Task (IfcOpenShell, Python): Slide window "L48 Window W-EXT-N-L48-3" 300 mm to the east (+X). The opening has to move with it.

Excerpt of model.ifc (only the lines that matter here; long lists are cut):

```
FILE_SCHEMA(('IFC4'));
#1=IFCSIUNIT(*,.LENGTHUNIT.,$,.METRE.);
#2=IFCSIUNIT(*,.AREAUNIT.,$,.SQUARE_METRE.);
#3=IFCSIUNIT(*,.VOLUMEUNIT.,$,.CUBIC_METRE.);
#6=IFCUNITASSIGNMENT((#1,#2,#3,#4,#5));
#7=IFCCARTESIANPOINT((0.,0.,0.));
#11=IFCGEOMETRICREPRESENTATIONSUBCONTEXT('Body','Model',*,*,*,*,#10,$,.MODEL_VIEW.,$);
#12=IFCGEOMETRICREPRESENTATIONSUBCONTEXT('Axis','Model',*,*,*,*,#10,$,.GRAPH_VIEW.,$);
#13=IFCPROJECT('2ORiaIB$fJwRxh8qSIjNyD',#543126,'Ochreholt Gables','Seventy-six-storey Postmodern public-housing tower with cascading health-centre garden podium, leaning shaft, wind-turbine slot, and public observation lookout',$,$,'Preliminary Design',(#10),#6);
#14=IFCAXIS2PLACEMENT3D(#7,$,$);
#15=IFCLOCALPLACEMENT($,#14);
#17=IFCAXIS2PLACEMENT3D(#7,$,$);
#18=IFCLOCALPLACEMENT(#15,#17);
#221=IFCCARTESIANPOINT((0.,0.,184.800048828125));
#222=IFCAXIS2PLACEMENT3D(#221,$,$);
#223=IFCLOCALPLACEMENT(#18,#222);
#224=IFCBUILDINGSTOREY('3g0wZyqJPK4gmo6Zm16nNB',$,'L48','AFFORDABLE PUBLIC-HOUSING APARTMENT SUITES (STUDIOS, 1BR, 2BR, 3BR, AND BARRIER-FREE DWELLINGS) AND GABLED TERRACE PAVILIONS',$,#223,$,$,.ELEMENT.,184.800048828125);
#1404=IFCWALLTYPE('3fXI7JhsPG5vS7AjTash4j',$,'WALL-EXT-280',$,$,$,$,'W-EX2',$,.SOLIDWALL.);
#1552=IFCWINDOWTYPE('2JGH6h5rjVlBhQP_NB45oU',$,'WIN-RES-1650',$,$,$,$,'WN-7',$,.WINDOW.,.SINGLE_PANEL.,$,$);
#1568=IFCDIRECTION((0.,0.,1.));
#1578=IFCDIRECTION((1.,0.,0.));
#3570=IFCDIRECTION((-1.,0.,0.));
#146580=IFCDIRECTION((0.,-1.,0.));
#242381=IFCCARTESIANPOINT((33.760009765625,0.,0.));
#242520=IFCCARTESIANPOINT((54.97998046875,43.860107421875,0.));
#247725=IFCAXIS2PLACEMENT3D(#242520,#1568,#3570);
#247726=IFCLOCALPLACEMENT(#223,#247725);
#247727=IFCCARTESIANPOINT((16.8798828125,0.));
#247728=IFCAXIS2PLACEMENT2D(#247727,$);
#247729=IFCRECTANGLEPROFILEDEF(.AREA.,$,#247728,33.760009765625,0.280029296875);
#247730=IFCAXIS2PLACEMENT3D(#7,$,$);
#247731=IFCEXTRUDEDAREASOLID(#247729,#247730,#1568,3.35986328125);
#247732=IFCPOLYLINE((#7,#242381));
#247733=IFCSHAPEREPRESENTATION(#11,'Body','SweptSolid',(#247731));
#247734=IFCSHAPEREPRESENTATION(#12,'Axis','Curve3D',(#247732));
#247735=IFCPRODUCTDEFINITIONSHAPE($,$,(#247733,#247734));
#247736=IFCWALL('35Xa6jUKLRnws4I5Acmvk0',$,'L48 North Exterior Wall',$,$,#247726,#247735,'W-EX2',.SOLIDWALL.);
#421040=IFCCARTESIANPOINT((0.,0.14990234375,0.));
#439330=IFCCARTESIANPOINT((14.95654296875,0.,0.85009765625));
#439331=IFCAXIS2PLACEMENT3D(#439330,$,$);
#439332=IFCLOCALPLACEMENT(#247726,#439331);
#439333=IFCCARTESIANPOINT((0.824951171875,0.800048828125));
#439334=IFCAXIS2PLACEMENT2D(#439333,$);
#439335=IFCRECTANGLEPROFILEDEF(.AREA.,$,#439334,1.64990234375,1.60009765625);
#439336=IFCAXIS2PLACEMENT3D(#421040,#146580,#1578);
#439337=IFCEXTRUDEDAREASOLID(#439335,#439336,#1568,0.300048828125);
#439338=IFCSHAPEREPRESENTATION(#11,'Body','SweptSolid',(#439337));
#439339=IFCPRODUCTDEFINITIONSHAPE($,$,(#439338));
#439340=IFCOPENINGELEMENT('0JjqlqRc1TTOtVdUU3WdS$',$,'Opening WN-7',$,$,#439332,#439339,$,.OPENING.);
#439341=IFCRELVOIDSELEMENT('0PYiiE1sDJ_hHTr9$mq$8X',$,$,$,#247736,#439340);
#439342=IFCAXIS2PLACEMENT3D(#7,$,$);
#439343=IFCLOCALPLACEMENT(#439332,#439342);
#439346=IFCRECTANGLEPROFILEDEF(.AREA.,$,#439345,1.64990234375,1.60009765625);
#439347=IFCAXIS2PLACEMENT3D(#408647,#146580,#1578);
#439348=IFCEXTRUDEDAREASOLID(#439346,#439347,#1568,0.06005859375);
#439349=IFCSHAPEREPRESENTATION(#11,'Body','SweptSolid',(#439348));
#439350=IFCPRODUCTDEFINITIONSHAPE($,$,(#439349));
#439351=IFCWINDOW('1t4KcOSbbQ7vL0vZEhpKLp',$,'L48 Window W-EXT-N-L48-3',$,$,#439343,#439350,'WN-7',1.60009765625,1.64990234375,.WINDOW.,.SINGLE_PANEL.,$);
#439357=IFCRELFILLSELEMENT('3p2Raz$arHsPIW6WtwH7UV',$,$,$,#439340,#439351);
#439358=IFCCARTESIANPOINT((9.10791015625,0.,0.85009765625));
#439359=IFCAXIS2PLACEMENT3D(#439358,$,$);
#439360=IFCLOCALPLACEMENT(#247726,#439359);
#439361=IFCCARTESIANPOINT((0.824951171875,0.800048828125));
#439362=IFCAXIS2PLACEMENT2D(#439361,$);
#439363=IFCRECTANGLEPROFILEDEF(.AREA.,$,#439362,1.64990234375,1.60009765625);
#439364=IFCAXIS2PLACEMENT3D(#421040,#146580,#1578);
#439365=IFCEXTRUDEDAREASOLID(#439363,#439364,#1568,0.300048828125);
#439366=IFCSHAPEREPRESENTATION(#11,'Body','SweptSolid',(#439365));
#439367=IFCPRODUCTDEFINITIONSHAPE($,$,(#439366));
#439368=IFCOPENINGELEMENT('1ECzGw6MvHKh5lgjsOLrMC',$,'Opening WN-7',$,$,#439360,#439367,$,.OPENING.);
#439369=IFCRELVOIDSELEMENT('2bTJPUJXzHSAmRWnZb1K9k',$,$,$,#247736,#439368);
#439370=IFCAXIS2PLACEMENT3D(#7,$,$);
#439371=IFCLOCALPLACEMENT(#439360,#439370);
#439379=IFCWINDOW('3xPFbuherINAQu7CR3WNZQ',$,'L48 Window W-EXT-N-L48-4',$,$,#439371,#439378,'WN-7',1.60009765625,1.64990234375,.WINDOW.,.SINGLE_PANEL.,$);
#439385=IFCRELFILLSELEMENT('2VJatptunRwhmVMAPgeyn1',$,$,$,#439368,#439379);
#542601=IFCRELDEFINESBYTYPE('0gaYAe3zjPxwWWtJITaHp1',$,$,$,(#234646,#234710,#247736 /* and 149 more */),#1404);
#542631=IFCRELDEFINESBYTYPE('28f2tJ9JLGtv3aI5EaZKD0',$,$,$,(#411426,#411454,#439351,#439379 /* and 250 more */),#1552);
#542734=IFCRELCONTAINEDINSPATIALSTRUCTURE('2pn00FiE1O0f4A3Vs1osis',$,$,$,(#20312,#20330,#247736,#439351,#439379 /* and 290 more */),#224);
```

```python
import ifcopenshell
import ifcopenshell.api.geometry
import ifcopenshell.util.placement

model = ifcopenshell.open("model.ifc")

window = model.by_guid("1t4KcOSbbQ7vL0vZEhpKLp")
opening = window.FillsVoids[0].RelatingOpeningElement
wall = opening.VoidsElements[0].RelatingBuildingElement

wall_matrix = ifcopenshell.util.placement.get_local_placement(wall.ObjectPlacement)
shift = wall_matrix[:3, 0] * -0.3
before = ifcopenshell.util.placement.get_local_placement(window.ObjectPlacement)[:3, 3].copy()

# The window is placed relative to its opening, so it follows when the opening moves.
matrix = ifcopenshell.util.placement.get_local_placement(opening.ObjectPlacement)
matrix[:3, 3] += shift
ifcopenshell.api.geometry.edit_object_placement(
    model, product=opening, matrix=matrix, is_si=False, should_transform_children=True
)

after = ifcopenshell.util.placement.get_local_placement(window.ObjectPlacement)[:3, 3]
print("window moved by", (after - before).round(3) + 0.0)

model.write("model_edited.ifc")
```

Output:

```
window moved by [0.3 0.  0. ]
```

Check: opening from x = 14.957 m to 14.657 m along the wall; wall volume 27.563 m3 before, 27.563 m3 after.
